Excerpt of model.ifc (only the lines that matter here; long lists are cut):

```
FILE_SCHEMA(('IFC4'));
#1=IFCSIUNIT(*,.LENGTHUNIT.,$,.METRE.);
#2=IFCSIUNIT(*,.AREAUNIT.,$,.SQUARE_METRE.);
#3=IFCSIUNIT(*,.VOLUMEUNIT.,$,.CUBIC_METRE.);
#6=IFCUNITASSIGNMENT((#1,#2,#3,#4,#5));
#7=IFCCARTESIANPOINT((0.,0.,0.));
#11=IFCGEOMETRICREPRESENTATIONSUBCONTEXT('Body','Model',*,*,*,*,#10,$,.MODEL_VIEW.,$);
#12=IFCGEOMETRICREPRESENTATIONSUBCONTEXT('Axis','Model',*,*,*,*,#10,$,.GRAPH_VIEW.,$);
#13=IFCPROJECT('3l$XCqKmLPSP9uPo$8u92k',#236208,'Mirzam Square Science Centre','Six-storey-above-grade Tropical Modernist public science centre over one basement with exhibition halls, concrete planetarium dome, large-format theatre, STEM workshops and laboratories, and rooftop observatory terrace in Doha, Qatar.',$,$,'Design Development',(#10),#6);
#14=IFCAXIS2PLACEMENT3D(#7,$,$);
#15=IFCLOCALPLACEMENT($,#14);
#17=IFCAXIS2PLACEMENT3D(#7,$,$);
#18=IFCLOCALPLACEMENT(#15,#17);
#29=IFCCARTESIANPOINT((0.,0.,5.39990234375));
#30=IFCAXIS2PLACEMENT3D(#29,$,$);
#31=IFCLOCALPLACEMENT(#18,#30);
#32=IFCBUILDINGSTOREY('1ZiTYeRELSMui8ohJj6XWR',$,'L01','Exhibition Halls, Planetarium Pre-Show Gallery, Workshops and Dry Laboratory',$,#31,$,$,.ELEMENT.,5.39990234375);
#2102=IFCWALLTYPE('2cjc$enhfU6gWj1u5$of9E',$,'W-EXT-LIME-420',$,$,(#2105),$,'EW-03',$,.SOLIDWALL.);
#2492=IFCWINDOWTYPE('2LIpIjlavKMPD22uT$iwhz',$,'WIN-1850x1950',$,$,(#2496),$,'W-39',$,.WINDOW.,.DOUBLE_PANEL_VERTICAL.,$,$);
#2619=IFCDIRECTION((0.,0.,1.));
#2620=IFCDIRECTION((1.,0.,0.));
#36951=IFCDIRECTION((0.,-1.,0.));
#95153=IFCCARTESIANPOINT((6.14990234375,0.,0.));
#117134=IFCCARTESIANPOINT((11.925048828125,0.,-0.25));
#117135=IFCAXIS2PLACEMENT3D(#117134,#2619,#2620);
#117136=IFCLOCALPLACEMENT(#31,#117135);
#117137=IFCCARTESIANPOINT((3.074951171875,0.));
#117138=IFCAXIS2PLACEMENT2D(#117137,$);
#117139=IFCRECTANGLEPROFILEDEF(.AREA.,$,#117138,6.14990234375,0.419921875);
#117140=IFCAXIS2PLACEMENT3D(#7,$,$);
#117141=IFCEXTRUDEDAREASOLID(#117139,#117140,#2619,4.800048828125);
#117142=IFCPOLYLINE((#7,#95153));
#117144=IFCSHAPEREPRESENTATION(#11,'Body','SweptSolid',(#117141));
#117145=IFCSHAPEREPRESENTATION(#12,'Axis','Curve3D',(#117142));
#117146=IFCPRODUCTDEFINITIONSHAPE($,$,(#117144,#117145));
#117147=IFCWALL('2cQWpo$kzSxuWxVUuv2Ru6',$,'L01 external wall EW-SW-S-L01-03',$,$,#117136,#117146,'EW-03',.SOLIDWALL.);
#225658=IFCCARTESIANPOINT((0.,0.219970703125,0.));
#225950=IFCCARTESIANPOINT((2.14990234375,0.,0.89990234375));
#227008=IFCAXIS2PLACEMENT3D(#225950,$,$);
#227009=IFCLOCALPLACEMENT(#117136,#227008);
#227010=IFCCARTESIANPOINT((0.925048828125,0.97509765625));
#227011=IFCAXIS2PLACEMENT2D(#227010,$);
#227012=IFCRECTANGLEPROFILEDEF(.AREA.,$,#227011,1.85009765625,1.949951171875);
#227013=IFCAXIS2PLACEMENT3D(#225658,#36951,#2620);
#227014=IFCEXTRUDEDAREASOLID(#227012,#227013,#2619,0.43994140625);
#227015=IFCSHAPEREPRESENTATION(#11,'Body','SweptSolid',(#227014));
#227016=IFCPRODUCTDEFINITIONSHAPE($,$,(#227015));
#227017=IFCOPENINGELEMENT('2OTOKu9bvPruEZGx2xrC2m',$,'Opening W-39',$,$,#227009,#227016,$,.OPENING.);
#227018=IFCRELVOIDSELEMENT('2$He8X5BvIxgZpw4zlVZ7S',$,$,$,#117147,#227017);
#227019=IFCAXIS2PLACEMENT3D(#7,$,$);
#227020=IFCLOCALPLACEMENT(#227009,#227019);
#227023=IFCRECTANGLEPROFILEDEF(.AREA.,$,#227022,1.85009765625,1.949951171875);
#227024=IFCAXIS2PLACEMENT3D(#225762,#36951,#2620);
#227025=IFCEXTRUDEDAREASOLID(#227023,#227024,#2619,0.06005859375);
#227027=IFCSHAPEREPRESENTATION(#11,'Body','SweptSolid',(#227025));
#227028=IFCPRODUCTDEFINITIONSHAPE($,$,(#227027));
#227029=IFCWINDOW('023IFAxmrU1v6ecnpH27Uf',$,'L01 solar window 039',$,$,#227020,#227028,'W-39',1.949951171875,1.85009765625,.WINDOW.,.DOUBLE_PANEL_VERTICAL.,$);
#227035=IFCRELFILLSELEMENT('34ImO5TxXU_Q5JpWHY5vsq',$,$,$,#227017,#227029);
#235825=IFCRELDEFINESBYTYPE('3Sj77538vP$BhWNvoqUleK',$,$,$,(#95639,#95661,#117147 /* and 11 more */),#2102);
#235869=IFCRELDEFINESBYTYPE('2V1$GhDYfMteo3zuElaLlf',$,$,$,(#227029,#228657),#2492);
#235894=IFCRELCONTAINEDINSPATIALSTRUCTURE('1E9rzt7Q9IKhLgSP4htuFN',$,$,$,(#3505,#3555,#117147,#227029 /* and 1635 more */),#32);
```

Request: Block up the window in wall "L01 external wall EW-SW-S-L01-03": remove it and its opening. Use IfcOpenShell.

```python
import ifcopenshell
import ifcopenshell.api.feature
import ifcopenshell.api.root
import ifcopenshell.geom
import ifcopenshell.util.shape

model = ifcopenshell.open("model.ifc")
settings = ifcopenshell.geom.settings()


def volume(element):
    """Net volume in cubic metres, openings subtracted."""
    shape = ifcopenshell.geom.create_shape(settings, element)
    return ifcopenshell.util.shape.get_volume(shape.geometry)


window = model.by_guid("023IFAxmrU1v6ecnpH27Uf")
opening = window.FillsVoids[0].RelatingOpeningElement
wall = opening.VoidsElements[0].RelatingBuildingElement
before = volume(wall)

ifcopenshell.api.root.remove_product(model, product=window)
ifcopenshell.api.feature.remove_feature(model, feature=opening)

after = volume(wall)

print(f"wall volume {before:.3f} -> {after:.3f} m3")

model.write("model_updated.ifc")
```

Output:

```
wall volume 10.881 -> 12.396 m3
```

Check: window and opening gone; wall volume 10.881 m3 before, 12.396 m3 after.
